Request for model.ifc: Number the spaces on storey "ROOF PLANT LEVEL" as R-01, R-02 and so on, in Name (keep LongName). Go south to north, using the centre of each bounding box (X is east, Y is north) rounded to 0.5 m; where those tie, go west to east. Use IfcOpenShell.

First a look at what the model holds.

```python
import ifcopenshell
import ifcopenshell.util.element
import ifcopenshell.util.placement

model = ifcopenshell.open("model.ifc")
print(model.schema)
storey = next(s for s in model.by_type("IfcBuildingStorey") if s.Name == "ROOF PLANT LEVEL")
spaces = [e for e in ifcopenshell.util.element.get_decomposition(storey) if e.is_a("IfcSpace")]
for e in sorted(spaces, key=lambda e: e.id()):
    origin = ifcopenshell.util.placement.get_local_placement(e.ObjectPlacement)[:3, 3]
    print(e.id(), e.Name, e.LongName, origin.round(2) + 0.0, sep=" | ")
```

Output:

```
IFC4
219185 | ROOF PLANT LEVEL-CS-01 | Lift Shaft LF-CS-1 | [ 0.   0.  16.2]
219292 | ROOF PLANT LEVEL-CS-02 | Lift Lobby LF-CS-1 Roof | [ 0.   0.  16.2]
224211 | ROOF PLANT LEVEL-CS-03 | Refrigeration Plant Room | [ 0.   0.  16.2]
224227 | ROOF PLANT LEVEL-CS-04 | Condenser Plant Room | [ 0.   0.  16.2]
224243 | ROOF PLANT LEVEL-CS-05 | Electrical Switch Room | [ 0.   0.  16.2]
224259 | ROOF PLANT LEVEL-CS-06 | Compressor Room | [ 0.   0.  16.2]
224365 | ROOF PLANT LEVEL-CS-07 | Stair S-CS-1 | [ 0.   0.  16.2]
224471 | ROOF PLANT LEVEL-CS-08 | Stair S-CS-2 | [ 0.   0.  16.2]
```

```python
import ifcopenshell
import ifcopenshell.geom
import ifcopenshell.util.element
import ifcopenshell.util.shape

model = ifcopenshell.open("model.ifc")
settings = ifcopenshell.geom.settings()
settings.set("use-world-coords", True)


def centre(element):
    shape = ifcopenshell.geom.create_shape(settings, element)
    return ifcopenshell.util.shape.get_bbox_centroid(shape.geometry)


storey = next(s for s in model.by_type("IfcBuildingStorey") if s.Name == "ROOF PLANT LEVEL")
spaces = [e for e in ifcopenshell.util.element.get_decomposition(storey) if e.is_a("IfcSpace")]

# Insertion points can sit at a corner or the storey origin, so sort by the geometry (in metres).
centres = {e: centre(e) for e in spaces}
spaces.sort(key=lambda e: (round(centres[e][1] / 0.5), centres[e][0]))

for i, e in enumerate(spaces, start=1):
    number = f"R-{i:02d}"
    e.Name = number
    print(e.id(), number)

model.write("model_updated.ifc")
```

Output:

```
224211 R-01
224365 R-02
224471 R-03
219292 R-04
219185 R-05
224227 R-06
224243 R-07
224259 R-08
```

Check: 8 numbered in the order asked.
